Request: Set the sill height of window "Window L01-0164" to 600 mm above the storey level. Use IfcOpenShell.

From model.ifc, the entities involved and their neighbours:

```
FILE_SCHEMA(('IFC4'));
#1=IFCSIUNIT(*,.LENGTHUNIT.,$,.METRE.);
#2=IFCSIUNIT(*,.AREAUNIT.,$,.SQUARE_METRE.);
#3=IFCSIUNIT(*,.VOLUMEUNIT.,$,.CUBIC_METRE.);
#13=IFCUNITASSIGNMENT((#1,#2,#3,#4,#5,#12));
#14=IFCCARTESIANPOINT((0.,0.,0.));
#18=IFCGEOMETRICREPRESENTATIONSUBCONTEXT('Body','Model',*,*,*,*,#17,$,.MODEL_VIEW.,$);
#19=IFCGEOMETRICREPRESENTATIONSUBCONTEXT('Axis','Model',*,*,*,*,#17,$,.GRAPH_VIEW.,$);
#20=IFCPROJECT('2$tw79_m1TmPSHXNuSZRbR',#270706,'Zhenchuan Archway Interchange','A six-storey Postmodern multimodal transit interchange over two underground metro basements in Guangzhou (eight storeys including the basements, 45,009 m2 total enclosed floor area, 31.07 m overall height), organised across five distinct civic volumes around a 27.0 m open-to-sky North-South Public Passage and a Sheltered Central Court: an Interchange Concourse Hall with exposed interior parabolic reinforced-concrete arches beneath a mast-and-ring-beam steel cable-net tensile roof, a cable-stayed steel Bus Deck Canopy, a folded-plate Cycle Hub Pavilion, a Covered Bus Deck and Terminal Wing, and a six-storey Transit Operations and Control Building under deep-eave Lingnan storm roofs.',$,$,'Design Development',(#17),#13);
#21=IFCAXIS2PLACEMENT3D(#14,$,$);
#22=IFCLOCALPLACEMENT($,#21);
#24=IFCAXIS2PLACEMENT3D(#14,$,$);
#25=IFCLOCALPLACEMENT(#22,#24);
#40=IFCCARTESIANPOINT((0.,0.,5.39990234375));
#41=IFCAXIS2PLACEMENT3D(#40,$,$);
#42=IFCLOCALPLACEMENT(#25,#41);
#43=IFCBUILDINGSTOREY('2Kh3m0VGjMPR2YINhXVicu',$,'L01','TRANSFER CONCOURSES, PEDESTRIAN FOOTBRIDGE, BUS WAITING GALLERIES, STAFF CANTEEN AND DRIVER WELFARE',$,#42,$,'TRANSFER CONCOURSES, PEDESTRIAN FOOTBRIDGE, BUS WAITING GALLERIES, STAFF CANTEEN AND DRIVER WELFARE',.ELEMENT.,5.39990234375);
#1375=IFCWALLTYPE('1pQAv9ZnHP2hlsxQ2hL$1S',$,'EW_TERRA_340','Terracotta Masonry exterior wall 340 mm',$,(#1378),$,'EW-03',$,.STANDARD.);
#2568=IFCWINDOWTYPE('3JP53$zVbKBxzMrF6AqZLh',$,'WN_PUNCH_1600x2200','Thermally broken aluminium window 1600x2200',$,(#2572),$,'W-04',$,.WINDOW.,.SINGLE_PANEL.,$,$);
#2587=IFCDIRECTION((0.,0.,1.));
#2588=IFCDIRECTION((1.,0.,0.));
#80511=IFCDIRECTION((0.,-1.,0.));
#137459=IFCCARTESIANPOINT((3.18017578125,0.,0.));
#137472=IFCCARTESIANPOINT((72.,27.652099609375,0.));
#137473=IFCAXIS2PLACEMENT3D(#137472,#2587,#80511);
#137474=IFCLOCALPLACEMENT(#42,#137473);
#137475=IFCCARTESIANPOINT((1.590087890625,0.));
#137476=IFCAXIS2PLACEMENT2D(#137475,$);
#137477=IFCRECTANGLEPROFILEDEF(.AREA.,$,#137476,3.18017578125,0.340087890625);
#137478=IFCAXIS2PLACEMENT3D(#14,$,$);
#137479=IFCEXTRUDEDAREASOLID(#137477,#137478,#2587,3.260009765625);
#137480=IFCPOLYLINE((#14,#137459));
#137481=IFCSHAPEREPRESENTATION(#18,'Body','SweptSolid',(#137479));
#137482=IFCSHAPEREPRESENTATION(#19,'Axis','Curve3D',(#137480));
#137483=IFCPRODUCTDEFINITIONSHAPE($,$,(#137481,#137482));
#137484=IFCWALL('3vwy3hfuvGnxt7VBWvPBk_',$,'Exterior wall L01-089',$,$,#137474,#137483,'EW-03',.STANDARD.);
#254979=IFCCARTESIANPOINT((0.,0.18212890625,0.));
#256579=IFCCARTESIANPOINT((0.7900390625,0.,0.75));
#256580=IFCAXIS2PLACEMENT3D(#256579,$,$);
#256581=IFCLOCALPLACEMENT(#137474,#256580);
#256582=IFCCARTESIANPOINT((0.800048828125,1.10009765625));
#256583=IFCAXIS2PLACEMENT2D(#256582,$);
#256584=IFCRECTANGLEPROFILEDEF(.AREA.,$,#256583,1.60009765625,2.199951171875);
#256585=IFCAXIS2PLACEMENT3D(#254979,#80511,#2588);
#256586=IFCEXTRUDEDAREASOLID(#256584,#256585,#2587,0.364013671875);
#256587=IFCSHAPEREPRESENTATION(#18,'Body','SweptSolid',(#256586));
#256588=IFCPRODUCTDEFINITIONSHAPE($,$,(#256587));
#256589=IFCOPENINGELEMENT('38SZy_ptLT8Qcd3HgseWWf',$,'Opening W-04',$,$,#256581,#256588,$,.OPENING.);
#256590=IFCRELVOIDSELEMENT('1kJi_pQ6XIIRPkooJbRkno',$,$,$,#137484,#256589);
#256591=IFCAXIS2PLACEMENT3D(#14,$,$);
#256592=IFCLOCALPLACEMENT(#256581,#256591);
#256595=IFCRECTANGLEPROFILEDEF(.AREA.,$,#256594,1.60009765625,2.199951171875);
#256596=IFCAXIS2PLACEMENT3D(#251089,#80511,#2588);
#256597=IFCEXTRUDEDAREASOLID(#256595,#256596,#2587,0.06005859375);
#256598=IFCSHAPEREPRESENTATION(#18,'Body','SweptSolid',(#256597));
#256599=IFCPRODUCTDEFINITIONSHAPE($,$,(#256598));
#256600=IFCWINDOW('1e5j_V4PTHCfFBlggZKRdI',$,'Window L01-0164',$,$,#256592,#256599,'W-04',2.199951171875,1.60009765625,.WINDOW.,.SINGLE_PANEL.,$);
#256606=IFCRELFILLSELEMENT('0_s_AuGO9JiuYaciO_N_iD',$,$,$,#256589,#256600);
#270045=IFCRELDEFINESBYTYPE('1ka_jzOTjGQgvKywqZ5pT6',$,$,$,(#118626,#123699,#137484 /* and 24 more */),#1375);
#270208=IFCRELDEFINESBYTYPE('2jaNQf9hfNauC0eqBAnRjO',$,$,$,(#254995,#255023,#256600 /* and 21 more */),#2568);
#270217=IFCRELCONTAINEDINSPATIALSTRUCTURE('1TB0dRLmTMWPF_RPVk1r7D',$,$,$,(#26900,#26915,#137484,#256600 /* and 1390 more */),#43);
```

```python
import numpy as np
import ifcopenshell
import ifcopenshell.api.geometry
import ifcopenshell.geom
import ifcopenshell.util.element
import ifcopenshell.util.placement
import ifcopenshell.util.shape
import ifcopenshell.util.unit

model = ifcopenshell.open("model.ifc")
unit_scale = ifcopenshell.util.unit.calculate_unit_scale(model)

window = model.by_guid("1e5j_V4PTHCfFBlggZKRdI")
opening = window.FillsVoids[0].RelatingOpeningElement
storey = ifcopenshell.util.element.get_container(window, ifc_class="IfcBuildingStorey")
level = ifcopenshell.util.placement.get_local_placement(storey.ObjectPlacement)[2, 3]

# The opening's origin need not be at the sill, so measure its lowest point.
shape = ifcopenshell.geom.create_shape(ifcopenshell.geom.settings(), opening)
bottom = ifcopenshell.util.shape.get_shape_bottom_elevation(shape, shape.geometry) / unit_scale
dz = level + 0.6 - bottom

shift = np.array([0.0, 0.0, dz])
# The window is placed relative to its opening, so it follows when the opening moves.
matrix = ifcopenshell.util.placement.get_local_placement(opening.ObjectPlacement)
matrix[:3, 3] += shift
ifcopenshell.api.geometry.edit_object_placement(
    model, product=opening, matrix=matrix, is_si=False, should_transform_children=True
)

print(f"moved by {dz * unit_scale:+.3f} m")

model.write("model_rev.ifc")
```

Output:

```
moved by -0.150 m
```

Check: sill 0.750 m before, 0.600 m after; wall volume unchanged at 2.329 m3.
